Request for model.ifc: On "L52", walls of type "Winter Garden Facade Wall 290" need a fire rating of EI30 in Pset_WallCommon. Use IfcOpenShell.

First a look at what the model holds.

```python
import ifcopenshell
import ifcopenshell.util.element

model = ifcopenshell.open("model.ifc")
print(model.schema)
storey = next(s for s in model.by_type("IfcBuildingStorey") if s.Name == "L52")
walls = [e for e in ifcopenshell.util.element.get_decomposition(storey) if e.is_a("IfcWall")]
seen = {}
for e in walls:
    element_type = ifcopenshell.util.element.get_type(e)
    key = (element_type.Name if element_type != e and element_type else None, ifcopenshell.util.element.get_pset(e, "Pset_WallCommon", "FireRating"))
    seen[key] = seen.get(key, 0) + 1
for (name, value), count in sorted(seen.items(), key=str):
    print(count, "x", name, "|", value)
```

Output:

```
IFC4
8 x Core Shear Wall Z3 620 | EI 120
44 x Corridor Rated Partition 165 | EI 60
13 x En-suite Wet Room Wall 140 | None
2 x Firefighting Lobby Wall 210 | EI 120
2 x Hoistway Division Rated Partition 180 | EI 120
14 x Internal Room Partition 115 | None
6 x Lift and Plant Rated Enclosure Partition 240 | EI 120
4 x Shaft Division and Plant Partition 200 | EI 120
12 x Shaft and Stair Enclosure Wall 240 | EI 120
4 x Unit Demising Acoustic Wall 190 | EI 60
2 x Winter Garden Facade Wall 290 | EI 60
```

```python
import ifcopenshell
import ifcopenshell.api.pset
import ifcopenshell.util.element

model = ifcopenshell.open("model.ifc")

storey = next(s for s in model.by_type("IfcBuildingStorey") if s.Name == "L52")
walls = [e for e in ifcopenshell.util.element.get_decomposition(storey) if e.is_a("IfcWall")]

count = 0
for e in walls:
    element_type = ifcopenshell.util.element.get_type(e)
    if element_type in (None, e) or element_type.Name != "Winter Garden Facade Wall 290":
        continue
    found = ifcopenshell.util.element.get_pset(e, "Pset_WallCommon", should_inherit=False)
    if found:
        pset = model.by_id(found["id"])
        if len(ifcopenshell.util.element.get_elements_by_pset(pset)) > 1:
            pset = ifcopenshell.api.pset.unshare_pset(model, products=[e], pset=pset)[0]
    else:
        pset = ifcopenshell.api.pset.add_pset(model, product=e, name="Pset_WallCommon")
    ifcopenshell.api.pset.edit_pset(model, pset=pset, properties={"FireRating": "EI30"})
    count += 1

print(count, "walls updated")

model.write("model_edited.ifc")
```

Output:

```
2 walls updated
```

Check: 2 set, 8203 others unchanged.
